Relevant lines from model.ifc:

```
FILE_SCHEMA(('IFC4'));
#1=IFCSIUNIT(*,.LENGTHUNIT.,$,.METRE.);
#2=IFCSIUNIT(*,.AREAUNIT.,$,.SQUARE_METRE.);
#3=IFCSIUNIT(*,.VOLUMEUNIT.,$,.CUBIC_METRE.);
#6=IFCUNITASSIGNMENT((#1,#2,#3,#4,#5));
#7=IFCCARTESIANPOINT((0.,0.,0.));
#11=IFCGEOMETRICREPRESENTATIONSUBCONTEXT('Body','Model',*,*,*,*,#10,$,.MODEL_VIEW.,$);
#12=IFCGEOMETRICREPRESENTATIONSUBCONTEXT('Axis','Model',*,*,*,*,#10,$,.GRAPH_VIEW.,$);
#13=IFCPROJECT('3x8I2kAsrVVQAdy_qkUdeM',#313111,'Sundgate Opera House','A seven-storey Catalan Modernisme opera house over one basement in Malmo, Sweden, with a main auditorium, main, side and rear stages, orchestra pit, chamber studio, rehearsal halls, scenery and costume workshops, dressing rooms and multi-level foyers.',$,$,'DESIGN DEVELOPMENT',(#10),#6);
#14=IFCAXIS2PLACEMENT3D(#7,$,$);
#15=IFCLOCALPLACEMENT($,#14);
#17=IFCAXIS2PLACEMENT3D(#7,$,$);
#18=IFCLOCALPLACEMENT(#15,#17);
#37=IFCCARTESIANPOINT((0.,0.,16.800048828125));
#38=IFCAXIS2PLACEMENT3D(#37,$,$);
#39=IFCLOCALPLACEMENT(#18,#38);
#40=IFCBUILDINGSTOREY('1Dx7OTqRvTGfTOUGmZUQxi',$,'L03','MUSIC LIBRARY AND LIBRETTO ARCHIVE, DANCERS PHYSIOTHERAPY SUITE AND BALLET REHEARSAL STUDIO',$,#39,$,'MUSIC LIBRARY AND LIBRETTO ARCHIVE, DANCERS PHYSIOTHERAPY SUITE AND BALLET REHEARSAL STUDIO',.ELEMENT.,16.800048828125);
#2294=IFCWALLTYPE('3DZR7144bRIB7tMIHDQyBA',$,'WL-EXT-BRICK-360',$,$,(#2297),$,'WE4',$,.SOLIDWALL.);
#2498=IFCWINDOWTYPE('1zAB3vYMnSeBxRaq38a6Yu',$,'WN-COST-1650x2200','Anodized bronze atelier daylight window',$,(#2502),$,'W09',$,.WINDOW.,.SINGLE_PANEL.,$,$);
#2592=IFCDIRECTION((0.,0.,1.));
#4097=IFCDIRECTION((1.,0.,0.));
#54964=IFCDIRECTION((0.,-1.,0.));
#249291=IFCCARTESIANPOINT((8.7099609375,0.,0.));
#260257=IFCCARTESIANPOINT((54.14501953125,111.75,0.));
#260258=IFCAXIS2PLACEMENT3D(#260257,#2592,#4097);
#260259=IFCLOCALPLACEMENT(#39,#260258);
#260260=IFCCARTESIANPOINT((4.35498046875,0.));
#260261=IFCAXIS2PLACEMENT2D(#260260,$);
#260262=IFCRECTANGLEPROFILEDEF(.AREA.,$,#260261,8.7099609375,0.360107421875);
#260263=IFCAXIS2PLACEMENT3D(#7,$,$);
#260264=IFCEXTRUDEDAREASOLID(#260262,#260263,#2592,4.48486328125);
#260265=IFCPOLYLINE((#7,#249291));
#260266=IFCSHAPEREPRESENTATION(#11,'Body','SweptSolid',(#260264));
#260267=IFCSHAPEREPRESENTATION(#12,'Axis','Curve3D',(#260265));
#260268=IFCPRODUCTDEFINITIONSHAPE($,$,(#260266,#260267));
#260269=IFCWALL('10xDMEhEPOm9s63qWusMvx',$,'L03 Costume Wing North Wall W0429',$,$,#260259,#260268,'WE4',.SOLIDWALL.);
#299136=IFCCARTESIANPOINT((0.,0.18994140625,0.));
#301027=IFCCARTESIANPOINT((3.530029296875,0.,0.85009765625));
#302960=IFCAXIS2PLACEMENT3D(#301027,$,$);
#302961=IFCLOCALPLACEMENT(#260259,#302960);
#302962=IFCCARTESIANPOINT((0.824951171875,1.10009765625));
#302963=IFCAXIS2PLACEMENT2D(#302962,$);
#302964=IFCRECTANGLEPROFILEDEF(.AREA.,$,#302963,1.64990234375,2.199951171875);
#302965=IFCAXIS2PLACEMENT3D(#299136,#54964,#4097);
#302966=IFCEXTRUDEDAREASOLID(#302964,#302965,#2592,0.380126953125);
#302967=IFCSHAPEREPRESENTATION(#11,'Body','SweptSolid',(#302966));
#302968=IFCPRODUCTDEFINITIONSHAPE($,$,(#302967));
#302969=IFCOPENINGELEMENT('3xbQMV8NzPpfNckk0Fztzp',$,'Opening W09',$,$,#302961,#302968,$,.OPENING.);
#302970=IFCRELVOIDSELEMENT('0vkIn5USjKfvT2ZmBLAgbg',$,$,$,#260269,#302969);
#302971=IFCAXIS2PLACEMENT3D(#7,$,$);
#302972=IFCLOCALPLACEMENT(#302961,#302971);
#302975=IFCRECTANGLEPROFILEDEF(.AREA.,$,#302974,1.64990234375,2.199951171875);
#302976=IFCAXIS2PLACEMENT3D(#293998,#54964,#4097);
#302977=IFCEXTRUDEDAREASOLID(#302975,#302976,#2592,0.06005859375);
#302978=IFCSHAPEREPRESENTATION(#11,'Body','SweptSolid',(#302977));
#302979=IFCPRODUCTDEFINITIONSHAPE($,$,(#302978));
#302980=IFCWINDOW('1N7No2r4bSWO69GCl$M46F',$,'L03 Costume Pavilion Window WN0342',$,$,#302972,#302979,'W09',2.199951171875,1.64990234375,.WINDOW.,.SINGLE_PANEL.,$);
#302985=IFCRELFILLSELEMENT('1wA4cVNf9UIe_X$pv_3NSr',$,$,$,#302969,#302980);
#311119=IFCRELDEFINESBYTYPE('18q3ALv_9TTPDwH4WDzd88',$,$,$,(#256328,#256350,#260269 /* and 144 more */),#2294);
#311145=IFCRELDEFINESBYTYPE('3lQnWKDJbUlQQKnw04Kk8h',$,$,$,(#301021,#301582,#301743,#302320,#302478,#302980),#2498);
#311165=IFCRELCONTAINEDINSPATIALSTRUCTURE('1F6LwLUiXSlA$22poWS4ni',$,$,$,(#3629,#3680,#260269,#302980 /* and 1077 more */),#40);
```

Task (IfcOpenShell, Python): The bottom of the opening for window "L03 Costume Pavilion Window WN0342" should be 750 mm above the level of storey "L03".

```python
import numpy as np
import ifcopenshell
import ifcopenshell.api.geometry
import ifcopenshell.geom
import ifcopenshell.util.element
import ifcopenshell.util.placement
import ifcopenshell.util.shape
import ifcopenshell.util.unit

model = ifcopenshell.open("model.ifc")
unit_scale = ifcopenshell.util.unit.calculate_unit_scale(model)

window = model.by_guid("1N7No2r4bSWO69GCl$M46F")
opening = window.FillsVoids[0].RelatingOpeningElement
storey = ifcopenshell.util.element.get_container(window, ifc_class="IfcBuildingStorey")
level = ifcopenshell.util.placement.get_local_placement(storey.ObjectPlacement)[2, 3]

# The opening's origin need not be at the sill, so measure its lowest point.
shape = ifcopenshell.geom.create_shape(ifcopenshell.geom.settings(), opening)
bottom = ifcopenshell.util.shape.get_shape_bottom_elevation(shape, shape.geometry) / unit_scale
dz = level + 0.75 - bottom

shift = np.array([0.0, 0.0, dz])
# The window is placed relative to its opening, so it follows when the opening moves.
matrix = ifcopenshell.util.placement.get_local_placement(opening.ObjectPlacement)
matrix[:3, 3] += shift
ifcopenshell.api.geometry.edit_object_placement(
    model, product=opening, matrix=matrix, is_si=False, should_transform_children=True
)

print(f"moved by {dz * unit_scale:+.3f} m")

model.write("model_rev.ifc")
```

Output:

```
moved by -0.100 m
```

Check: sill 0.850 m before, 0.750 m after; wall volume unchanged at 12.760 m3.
